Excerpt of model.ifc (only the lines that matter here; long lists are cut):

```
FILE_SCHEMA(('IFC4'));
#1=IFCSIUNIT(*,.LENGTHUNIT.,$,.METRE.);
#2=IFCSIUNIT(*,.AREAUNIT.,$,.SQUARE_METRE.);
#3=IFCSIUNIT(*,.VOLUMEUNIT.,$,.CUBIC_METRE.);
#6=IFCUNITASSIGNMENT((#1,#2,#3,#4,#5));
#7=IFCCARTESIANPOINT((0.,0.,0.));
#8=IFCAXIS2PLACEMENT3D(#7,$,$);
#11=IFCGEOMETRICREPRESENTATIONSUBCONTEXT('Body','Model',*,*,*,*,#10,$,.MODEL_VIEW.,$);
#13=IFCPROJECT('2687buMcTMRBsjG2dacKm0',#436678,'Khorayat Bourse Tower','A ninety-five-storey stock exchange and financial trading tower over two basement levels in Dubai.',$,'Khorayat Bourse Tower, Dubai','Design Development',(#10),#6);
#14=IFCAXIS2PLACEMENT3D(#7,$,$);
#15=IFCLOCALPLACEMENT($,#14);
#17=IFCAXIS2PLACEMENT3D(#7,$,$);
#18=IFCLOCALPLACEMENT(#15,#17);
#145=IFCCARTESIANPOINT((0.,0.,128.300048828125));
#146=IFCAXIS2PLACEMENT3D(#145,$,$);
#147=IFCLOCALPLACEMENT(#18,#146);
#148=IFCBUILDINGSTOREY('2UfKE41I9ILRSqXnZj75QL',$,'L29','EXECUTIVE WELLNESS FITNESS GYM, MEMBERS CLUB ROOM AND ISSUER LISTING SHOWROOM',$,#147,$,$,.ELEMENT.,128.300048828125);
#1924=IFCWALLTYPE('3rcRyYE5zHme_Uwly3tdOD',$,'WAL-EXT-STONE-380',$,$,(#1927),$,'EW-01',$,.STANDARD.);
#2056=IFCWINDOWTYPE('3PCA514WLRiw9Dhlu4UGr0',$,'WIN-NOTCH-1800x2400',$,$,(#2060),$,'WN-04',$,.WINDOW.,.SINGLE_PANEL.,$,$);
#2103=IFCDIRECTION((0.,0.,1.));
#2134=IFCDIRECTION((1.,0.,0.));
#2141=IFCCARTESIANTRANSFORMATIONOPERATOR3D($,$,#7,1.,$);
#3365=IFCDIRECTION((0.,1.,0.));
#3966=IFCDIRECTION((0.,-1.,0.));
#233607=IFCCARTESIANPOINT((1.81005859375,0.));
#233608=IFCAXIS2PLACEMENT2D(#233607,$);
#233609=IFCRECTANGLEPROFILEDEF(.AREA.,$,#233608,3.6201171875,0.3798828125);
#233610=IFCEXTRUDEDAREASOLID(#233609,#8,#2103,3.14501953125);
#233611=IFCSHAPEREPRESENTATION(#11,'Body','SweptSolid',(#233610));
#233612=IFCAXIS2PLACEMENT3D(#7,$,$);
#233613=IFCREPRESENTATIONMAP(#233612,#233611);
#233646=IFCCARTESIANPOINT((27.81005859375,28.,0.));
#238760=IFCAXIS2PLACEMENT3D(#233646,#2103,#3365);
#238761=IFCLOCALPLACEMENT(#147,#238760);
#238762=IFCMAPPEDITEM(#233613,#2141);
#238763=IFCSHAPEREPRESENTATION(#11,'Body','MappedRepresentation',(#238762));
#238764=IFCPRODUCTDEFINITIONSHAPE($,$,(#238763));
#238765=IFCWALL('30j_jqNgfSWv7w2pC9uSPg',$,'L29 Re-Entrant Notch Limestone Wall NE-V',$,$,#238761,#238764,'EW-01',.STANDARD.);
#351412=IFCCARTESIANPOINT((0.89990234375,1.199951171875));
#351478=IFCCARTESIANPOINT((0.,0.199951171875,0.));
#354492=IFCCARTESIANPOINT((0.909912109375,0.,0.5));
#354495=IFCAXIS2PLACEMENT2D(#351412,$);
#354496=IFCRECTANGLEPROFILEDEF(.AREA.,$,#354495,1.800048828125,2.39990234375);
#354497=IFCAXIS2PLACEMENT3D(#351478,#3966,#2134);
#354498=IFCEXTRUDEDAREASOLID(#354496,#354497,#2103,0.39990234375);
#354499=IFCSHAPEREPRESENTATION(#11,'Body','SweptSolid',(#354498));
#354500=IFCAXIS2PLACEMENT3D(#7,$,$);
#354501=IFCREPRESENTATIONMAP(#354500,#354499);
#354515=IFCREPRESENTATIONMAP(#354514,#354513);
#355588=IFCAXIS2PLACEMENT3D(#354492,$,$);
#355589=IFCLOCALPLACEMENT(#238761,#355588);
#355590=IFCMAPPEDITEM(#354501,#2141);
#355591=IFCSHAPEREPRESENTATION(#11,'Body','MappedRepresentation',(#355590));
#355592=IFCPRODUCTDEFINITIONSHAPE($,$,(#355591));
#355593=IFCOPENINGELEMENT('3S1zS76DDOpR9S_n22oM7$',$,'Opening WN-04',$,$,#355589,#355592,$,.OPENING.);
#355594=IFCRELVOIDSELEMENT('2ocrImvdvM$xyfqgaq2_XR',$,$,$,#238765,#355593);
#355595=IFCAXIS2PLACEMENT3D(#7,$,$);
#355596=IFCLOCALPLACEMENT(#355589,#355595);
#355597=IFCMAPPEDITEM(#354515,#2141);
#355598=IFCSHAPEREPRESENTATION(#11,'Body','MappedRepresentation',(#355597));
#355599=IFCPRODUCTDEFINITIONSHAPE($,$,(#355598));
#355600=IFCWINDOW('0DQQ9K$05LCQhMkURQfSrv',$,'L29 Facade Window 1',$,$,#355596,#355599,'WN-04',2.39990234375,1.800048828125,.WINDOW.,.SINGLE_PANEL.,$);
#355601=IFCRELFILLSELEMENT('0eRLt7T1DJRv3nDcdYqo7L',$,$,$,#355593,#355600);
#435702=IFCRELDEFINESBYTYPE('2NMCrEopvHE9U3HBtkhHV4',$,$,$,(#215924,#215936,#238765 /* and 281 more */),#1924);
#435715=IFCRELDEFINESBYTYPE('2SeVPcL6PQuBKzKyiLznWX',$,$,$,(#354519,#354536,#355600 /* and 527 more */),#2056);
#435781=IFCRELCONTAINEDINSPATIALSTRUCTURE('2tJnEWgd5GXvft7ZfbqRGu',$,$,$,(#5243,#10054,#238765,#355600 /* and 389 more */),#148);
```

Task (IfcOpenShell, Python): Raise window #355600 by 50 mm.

```python
import numpy as np
import ifcopenshell
import ifcopenshell.api.geometry
import ifcopenshell.util.placement
import ifcopenshell.util.unit

model = ifcopenshell.open("model.ifc")
unit_scale = ifcopenshell.util.unit.calculate_unit_scale(model)

window = model.by_id(355600)
opening = window.FillsVoids[0].RelatingOpeningElement
dz = 0.05

shift = np.array([0.0, 0.0, dz])
# The window is placed relative to its opening, so it follows when the opening moves.
matrix = ifcopenshell.util.placement.get_local_placement(opening.ObjectPlacement)
matrix[:3, 3] += shift
ifcopenshell.api.geometry.edit_object_placement(
    model, product=opening, matrix=matrix, is_si=False, should_transform_children=True
)

print(f"moved by {dz * unit_scale:+.3f} m")

model.write("model_updated.ifc")
```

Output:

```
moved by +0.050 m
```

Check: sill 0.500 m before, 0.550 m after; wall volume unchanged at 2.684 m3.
